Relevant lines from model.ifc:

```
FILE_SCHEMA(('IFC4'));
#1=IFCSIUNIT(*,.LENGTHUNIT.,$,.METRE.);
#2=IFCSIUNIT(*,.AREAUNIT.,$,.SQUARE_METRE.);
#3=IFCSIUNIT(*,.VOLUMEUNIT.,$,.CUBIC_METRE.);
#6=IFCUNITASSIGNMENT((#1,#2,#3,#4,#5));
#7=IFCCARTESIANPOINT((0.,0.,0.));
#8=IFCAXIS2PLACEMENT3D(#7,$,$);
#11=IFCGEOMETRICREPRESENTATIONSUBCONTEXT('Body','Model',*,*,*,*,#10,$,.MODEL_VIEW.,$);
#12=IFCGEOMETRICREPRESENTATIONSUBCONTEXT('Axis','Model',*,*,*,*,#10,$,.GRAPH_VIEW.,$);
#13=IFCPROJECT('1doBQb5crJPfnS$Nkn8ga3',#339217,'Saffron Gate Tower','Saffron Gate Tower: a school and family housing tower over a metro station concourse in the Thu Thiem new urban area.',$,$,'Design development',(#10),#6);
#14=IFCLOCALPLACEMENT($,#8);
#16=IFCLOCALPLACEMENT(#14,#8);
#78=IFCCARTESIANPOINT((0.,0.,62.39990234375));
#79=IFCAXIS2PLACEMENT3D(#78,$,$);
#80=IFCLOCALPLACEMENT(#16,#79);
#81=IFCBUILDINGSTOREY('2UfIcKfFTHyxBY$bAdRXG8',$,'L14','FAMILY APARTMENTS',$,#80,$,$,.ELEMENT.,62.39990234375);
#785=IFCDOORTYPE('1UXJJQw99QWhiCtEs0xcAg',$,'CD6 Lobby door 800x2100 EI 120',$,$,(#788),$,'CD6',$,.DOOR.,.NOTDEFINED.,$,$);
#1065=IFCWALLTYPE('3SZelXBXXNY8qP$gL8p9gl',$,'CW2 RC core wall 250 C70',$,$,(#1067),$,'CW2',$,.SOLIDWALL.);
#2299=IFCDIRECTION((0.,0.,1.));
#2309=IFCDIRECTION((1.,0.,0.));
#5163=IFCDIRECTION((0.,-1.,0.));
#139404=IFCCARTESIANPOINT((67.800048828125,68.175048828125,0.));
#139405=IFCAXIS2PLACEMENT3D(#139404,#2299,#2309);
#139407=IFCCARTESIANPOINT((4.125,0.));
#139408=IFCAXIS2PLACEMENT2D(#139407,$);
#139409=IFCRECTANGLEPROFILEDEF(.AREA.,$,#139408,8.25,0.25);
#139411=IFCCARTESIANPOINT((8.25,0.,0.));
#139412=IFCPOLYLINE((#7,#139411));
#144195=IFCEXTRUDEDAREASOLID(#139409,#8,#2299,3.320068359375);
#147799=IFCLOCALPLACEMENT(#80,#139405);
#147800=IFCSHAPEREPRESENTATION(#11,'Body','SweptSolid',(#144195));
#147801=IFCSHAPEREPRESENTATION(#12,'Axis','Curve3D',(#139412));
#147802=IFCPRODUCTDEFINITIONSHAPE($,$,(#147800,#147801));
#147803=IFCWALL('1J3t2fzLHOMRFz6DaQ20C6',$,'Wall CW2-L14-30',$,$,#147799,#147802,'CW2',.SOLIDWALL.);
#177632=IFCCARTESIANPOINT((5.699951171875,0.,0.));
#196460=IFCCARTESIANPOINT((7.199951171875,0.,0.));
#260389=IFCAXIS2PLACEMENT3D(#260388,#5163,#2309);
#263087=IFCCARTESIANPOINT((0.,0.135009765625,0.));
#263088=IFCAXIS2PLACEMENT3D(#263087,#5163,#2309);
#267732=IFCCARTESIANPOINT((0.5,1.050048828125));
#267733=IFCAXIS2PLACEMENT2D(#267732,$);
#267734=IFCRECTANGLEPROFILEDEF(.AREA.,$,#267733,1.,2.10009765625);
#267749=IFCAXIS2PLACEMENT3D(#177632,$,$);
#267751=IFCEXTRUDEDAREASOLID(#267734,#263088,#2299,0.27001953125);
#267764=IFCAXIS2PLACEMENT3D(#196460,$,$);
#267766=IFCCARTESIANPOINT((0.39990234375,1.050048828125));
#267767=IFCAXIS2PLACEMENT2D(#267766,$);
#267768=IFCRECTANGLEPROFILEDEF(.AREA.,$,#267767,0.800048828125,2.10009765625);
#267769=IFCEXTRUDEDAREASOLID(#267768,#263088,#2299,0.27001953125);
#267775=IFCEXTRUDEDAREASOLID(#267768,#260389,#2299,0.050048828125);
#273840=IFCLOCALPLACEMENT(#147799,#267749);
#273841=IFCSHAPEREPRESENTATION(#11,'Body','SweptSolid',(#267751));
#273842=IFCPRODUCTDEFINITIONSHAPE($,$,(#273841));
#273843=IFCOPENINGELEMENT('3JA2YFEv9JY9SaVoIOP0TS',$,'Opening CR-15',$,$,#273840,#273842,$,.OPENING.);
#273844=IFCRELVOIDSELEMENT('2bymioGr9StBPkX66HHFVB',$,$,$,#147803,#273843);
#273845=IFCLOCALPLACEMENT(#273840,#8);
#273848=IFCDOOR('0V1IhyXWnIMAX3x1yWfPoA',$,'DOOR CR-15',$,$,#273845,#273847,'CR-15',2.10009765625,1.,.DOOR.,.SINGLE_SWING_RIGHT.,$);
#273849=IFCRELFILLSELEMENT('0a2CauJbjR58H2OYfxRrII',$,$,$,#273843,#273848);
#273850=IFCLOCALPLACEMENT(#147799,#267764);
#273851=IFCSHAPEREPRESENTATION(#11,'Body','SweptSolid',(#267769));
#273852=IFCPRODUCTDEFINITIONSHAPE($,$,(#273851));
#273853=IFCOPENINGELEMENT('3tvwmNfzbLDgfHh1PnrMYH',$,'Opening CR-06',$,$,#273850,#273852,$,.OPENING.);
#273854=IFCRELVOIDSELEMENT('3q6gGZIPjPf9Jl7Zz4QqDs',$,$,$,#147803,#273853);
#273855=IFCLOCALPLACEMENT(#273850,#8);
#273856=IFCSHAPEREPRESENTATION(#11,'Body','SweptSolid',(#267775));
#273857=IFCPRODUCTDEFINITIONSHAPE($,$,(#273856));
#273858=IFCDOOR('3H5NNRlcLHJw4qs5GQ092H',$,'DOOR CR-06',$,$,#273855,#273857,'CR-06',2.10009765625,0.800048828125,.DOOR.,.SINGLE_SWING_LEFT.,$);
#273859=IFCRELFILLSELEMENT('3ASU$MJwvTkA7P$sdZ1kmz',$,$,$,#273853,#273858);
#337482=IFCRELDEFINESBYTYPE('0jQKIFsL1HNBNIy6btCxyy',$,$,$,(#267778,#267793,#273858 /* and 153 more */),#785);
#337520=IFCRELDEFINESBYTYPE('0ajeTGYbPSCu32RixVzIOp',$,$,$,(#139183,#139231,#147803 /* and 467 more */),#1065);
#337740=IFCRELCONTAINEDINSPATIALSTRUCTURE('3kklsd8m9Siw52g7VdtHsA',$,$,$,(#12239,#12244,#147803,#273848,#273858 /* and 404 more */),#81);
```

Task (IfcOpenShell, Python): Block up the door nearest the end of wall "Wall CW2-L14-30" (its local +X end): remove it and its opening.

```python
import ifcopenshell
import ifcopenshell.api.feature
import ifcopenshell.api.root
import ifcopenshell.geom
import ifcopenshell.util.shape

model = ifcopenshell.open("model.ifc")
settings = ifcopenshell.geom.settings()


def volume(element):
    """Net volume in cubic metres, openings subtracted."""
    shape = ifcopenshell.geom.create_shape(settings, element)
    return ifcopenshell.util.shape.get_volume(shape.geometry)


door = model.by_guid("3H5NNRlcLHJw4qs5GQ092H")
opening = door.FillsVoids[0].RelatingOpeningElement
wall = opening.VoidsElements[0].RelatingBuildingElement
before = volume(wall)

ifcopenshell.api.root.remove_product(model, product=door)
ifcopenshell.api.feature.remove_feature(model, feature=opening)

after = volume(wall)

print(f"wall volume {before:.3f} -> {after:.3f} m3")

model.write("model_rev.ifc")
```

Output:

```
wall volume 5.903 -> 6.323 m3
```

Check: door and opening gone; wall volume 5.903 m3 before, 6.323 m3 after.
